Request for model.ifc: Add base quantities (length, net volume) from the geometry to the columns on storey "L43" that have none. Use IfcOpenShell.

First a look at what the model holds.

```python
import ifcopenshell
import ifcopenshell.util.element
import ifcopenshell.util.unit

model = ifcopenshell.open("model.ifc")
print(model.schema)
for unit_type in ("LENGTHUNIT", "AREAUNIT", "VOLUMEUNIT"):
    print(unit_type, ifcopenshell.util.unit.calculate_unit_scale(model, unit_type))
storey = next(s for s in model.by_type("IfcBuildingStorey") if s.Name == "L43")
columns = [e for e in ifcopenshell.util.element.get_decomposition(storey) if e.is_a("IfcColumn")]
for e in sorted(columns, key=lambda e: e.id()):
    print(e.id(), e.is_a(), e.Name, list(ifcopenshell.util.element.get_psets(e, qtos_only=True)), sep=" | ")
```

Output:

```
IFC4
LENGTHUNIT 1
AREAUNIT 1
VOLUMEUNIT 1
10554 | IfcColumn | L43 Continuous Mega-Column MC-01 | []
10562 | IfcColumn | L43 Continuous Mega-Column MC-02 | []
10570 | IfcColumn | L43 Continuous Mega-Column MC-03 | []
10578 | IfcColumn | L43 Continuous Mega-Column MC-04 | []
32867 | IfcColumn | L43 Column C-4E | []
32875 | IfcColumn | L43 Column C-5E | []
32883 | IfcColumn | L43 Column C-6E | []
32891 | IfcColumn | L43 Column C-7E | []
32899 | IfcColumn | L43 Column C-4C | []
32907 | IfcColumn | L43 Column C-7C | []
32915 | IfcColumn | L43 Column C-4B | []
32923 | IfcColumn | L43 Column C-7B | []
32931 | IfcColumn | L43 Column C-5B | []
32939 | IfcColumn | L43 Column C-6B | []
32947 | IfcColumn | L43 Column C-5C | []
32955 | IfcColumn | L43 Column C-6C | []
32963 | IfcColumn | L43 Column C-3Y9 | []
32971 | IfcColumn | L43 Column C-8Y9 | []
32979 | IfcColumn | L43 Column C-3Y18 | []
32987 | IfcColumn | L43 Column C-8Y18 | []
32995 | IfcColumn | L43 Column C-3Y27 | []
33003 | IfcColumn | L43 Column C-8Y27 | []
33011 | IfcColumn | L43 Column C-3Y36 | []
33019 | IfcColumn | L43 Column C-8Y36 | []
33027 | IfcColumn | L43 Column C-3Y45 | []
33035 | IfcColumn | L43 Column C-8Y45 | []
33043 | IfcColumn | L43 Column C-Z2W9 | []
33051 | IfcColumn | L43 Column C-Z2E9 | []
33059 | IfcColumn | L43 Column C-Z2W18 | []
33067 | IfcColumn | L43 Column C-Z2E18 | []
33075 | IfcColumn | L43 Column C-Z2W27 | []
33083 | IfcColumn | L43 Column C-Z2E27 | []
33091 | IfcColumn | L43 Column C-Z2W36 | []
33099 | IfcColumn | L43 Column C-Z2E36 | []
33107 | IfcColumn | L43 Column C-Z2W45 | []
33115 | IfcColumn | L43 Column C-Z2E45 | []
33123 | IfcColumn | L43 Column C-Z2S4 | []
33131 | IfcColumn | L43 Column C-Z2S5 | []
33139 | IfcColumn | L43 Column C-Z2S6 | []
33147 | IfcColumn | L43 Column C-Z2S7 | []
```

```python
import ifcopenshell
import ifcopenshell.api.pset
import ifcopenshell.geom
import ifcopenshell.util.element
import ifcopenshell.util.shape
import ifcopenshell.util.unit

model = ifcopenshell.open("model.ifc")
unit_scale = ifcopenshell.util.unit.calculate_unit_scale(model)
volume_scale = ifcopenshell.util.unit.calculate_unit_scale(model, "VOLUMEUNIT")
settings = ifcopenshell.geom.settings()

storey = next(s for s in model.by_type("IfcBuildingStorey") if s.Name == "L43")
columns = [e for e in ifcopenshell.util.element.get_decomposition(storey) if e.is_a("IfcColumn")]

for e in sorted(columns, key=lambda e: e.id()):
    if ifcopenshell.util.element.get_psets(e, qtos_only=True, should_inherit=False):
        continue
    # Geometry comes back in metres, in the element's own axes.
    shape = ifcopenshell.geom.create_shape(settings, e)
    values = {
        "Length": ifcopenshell.util.shape.get_z(shape.geometry) / unit_scale,
        "NetVolume": ifcopenshell.util.shape.get_volume(shape.geometry) / volume_scale,
    }
    qto = ifcopenshell.api.pset.add_qto(model, product=e, name="Qto_ColumnBaseQuantities")
    ifcopenshell.api.pset.edit_qto(model, qto=qto, properties=values)
    print(e.id(), {k: round(v, 3) for k, v in values.items()})

model.write("model_updated.ifc")
```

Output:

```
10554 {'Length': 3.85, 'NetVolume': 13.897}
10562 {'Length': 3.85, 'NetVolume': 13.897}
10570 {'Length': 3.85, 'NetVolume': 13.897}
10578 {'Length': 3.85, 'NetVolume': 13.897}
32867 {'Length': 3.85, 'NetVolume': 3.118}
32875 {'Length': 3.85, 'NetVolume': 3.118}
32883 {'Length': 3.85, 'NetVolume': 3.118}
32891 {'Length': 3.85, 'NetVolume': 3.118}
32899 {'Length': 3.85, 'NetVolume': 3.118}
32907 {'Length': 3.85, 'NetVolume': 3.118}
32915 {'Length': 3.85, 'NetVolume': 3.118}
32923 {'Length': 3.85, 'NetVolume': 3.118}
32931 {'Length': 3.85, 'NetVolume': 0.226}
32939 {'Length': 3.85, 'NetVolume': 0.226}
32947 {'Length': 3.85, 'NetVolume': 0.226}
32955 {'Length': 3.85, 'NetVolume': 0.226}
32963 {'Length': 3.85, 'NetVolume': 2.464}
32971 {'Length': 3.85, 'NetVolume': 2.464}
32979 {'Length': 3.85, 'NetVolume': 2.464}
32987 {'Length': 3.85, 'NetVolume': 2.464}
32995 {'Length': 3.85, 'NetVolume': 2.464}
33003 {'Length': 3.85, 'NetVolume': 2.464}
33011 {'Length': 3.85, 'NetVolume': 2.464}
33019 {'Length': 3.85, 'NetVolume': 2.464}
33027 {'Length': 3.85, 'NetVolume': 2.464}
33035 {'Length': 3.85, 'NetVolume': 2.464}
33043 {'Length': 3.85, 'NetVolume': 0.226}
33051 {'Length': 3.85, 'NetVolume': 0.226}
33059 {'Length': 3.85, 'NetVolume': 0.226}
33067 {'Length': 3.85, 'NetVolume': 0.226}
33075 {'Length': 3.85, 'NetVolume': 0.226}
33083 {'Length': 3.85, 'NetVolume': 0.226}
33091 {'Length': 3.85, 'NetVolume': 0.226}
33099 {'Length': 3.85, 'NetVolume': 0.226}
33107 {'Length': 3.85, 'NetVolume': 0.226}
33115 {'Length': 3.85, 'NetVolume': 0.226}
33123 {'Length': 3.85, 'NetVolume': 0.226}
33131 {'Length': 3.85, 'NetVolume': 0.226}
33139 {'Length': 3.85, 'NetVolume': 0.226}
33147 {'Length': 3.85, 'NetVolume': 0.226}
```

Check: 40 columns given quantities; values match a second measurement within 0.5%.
